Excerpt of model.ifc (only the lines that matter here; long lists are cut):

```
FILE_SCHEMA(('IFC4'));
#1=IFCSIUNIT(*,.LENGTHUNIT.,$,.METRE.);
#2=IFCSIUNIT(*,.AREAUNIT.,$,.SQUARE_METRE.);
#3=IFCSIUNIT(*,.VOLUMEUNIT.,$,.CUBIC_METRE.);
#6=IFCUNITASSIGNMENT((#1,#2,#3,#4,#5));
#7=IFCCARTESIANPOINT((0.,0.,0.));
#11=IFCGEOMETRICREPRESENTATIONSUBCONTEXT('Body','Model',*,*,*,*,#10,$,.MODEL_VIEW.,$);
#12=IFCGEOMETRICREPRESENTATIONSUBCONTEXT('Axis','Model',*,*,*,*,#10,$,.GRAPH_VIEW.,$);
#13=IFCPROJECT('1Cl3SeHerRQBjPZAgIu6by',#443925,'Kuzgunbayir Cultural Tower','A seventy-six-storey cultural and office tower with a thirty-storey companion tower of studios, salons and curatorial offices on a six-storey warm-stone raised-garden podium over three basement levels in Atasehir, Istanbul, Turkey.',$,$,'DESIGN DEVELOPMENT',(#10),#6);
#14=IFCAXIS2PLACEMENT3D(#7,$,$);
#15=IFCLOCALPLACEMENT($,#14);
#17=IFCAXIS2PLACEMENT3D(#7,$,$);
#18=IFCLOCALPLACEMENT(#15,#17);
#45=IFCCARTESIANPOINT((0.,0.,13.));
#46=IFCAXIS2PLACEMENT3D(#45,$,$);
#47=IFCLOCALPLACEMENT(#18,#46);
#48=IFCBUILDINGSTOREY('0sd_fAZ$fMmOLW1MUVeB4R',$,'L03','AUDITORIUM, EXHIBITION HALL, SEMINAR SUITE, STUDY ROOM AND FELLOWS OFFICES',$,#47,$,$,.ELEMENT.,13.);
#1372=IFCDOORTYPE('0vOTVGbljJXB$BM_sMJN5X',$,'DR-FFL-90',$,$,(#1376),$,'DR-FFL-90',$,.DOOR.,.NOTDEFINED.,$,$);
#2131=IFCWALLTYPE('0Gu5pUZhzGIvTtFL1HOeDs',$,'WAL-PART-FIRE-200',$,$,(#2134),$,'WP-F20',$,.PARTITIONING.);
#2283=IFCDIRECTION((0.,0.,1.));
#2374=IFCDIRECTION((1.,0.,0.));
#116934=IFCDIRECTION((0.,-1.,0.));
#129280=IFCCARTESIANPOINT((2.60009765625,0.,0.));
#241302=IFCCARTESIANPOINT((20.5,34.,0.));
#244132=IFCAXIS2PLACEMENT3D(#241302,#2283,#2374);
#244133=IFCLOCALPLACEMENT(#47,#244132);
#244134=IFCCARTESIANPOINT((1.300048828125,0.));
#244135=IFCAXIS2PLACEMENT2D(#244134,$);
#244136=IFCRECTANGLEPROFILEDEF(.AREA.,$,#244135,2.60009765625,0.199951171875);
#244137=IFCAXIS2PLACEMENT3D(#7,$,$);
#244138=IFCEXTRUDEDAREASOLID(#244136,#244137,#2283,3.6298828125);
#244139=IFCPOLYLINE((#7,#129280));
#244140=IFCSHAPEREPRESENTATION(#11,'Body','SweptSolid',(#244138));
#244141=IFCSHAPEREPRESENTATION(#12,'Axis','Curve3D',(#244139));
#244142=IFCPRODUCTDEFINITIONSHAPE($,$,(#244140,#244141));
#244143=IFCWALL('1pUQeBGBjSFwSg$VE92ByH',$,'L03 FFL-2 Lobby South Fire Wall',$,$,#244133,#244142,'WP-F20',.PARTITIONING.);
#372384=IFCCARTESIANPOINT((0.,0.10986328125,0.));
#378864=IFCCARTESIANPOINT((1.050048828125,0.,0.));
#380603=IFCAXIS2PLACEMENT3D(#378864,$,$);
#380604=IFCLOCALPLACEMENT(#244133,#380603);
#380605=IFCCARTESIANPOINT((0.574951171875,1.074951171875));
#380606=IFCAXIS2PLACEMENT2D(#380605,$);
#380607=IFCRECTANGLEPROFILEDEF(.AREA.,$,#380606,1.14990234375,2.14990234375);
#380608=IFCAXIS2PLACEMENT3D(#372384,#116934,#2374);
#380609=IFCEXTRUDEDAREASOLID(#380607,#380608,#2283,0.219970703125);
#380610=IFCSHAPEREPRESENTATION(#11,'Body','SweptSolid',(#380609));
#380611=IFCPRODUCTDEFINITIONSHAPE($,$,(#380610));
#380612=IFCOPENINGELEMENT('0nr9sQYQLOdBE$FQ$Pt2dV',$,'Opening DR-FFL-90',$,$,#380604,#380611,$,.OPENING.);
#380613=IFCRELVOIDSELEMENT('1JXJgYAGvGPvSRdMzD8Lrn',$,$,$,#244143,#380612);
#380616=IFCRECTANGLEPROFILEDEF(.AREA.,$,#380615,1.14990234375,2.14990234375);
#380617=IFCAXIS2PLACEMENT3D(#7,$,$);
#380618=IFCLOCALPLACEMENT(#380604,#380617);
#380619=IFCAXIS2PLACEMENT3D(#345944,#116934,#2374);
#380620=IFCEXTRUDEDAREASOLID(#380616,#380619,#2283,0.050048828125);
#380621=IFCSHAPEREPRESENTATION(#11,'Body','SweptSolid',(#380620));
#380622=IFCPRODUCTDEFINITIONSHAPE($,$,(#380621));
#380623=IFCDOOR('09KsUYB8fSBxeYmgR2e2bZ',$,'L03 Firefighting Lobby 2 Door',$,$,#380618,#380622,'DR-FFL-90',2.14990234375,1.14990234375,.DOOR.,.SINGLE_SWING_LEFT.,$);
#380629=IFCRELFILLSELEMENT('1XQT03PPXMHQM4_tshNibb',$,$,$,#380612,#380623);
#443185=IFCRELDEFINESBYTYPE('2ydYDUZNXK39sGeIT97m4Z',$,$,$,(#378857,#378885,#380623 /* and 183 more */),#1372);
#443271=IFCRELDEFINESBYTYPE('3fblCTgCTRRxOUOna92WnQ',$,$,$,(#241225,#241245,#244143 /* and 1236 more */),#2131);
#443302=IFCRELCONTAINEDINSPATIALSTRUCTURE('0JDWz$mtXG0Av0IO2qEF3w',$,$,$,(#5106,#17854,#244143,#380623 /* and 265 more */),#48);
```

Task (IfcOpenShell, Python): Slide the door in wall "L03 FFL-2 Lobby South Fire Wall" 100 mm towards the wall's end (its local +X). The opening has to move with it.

```python
import ifcopenshell
import ifcopenshell.api.geometry
import ifcopenshell.util.placement
import ifcopenshell.util.unit

model = ifcopenshell.open("model.ifc")
unit_scale = ifcopenshell.util.unit.calculate_unit_scale(model)

door = model.by_guid("09KsUYB8fSBxeYmgR2e2bZ")
opening = door.FillsVoids[0].RelatingOpeningElement
wall = opening.VoidsElements[0].RelatingBuildingElement

wall_matrix = ifcopenshell.util.placement.get_local_placement(wall.ObjectPlacement)
shift = wall_matrix[:3, 0] * 0.1 / unit_scale
before = ifcopenshell.util.placement.get_local_placement(door.ObjectPlacement)[:3, 3].copy()

# The door is placed relative to its opening, so it follows when the opening moves.
matrix = ifcopenshell.util.placement.get_local_placement(opening.ObjectPlacement)
matrix[:3, 3] += shift
ifcopenshell.api.geometry.edit_object_placement(
    model, product=opening, matrix=matrix, is_si=False, should_transform_children=True
)

after = ifcopenshell.util.placement.get_local_placement(door.ObjectPlacement)[:3, 3]
print("door moved by", (after - before).round(3) + 0.0)

model.write("model_updated.ifc")
```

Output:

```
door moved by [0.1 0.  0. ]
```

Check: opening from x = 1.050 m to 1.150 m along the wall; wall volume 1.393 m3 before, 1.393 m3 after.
